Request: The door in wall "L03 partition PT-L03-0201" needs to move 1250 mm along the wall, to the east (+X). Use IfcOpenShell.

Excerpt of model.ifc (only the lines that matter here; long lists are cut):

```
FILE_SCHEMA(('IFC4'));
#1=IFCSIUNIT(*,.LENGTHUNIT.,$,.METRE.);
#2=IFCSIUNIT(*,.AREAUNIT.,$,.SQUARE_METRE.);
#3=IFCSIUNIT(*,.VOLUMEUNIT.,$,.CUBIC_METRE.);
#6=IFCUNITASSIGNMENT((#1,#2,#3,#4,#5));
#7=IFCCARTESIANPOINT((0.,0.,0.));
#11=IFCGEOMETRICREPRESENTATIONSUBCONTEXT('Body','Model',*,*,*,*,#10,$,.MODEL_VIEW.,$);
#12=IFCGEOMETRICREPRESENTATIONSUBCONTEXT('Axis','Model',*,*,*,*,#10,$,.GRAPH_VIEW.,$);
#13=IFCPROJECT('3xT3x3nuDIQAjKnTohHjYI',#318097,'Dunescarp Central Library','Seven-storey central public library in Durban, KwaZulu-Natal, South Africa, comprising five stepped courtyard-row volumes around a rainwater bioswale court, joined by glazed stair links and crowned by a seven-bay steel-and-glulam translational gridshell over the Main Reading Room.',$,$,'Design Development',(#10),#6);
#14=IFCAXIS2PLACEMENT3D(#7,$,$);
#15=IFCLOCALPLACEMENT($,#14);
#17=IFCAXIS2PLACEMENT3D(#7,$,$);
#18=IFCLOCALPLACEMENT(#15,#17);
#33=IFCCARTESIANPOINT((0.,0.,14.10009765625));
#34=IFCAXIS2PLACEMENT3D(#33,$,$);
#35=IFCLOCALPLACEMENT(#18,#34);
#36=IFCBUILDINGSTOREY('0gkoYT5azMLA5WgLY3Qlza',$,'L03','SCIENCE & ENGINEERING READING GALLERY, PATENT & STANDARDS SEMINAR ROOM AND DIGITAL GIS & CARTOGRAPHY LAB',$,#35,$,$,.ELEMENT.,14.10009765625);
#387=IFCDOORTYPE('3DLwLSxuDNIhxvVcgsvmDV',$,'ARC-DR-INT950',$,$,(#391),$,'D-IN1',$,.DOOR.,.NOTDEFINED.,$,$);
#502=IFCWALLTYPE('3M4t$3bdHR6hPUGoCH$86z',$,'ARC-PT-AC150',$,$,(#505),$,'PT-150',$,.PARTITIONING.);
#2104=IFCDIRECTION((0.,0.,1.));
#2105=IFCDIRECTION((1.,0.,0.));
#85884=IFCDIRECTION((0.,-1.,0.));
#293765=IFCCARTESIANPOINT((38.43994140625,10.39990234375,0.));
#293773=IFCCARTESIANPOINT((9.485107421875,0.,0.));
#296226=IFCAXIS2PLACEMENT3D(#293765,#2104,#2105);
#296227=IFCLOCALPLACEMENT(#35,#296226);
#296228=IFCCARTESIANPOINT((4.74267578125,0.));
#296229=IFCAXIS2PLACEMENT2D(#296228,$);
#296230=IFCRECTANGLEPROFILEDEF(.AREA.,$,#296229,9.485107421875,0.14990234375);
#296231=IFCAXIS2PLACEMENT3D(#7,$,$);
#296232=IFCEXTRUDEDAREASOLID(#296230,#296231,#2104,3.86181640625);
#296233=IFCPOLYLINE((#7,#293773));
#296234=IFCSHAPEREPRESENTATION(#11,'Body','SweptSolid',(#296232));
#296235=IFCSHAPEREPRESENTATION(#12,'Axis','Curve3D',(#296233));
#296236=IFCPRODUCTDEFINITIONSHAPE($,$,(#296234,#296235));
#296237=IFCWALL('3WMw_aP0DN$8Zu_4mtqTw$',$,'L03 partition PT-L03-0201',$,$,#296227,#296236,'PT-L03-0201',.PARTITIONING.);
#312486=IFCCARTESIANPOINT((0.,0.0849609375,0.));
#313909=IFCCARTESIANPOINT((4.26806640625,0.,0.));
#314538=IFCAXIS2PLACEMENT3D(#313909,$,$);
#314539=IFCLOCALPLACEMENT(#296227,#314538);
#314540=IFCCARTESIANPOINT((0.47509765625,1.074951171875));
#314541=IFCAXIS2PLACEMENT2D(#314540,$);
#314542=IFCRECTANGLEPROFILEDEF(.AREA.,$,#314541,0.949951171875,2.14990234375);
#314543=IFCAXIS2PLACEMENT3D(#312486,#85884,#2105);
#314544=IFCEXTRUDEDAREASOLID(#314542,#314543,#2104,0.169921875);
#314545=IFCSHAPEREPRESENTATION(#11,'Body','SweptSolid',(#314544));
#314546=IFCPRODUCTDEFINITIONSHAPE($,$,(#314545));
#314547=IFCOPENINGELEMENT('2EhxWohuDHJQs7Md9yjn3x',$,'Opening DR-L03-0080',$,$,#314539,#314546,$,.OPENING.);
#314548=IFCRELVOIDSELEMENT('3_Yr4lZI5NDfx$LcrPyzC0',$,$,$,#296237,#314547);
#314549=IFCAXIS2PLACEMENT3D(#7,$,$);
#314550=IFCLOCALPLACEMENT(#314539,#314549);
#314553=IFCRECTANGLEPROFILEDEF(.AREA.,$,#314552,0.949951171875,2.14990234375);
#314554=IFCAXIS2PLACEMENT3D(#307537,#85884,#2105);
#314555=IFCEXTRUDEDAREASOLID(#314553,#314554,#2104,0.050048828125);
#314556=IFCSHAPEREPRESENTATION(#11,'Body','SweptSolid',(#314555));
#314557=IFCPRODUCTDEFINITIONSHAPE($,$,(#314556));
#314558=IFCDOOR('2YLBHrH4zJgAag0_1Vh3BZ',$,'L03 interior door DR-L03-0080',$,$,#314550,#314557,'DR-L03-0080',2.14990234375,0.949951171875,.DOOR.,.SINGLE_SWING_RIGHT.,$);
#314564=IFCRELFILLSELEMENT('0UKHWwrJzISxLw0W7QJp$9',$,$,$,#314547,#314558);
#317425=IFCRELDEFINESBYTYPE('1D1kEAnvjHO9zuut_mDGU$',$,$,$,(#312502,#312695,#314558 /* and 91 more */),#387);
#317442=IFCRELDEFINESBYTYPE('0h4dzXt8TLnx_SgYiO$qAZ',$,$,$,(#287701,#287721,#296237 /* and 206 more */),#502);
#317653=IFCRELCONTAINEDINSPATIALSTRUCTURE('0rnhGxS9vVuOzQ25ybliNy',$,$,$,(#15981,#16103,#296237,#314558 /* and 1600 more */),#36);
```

```python
import ifcopenshell
import ifcopenshell.api.geometry
import ifcopenshell.util.placement
import ifcopenshell.util.unit

model = ifcopenshell.open("model.ifc")
unit_scale = ifcopenshell.util.unit.calculate_unit_scale(model)

door = model.by_guid("2YLBHrH4zJgAag0_1Vh3BZ")
opening = door.FillsVoids[0].RelatingOpeningElement
wall = opening.VoidsElements[0].RelatingBuildingElement

wall_matrix = ifcopenshell.util.placement.get_local_placement(wall.ObjectPlacement)
shift = wall_matrix[:3, 0] * 1.25 / unit_scale
before = ifcopenshell.util.placement.get_local_placement(door.ObjectPlacement)[:3, 3].copy()

# The door is placed relative to its opening, so it follows when the opening moves.
matrix = ifcopenshell.util.placement.get_local_placement(opening.ObjectPlacement)
matrix[:3, 3] += shift
ifcopenshell.api.geometry.edit_object_placement(
    model, product=opening, matrix=matrix, is_si=False, should_transform_children=True
)

after = ifcopenshell.util.placement.get_local_placement(door.ObjectPlacement)[:3, 3]
print("door moved by", (after - before).round(3) + 0.0)

model.write("model-out.ifc")
```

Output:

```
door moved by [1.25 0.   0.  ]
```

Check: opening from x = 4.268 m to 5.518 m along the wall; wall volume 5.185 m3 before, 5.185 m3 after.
